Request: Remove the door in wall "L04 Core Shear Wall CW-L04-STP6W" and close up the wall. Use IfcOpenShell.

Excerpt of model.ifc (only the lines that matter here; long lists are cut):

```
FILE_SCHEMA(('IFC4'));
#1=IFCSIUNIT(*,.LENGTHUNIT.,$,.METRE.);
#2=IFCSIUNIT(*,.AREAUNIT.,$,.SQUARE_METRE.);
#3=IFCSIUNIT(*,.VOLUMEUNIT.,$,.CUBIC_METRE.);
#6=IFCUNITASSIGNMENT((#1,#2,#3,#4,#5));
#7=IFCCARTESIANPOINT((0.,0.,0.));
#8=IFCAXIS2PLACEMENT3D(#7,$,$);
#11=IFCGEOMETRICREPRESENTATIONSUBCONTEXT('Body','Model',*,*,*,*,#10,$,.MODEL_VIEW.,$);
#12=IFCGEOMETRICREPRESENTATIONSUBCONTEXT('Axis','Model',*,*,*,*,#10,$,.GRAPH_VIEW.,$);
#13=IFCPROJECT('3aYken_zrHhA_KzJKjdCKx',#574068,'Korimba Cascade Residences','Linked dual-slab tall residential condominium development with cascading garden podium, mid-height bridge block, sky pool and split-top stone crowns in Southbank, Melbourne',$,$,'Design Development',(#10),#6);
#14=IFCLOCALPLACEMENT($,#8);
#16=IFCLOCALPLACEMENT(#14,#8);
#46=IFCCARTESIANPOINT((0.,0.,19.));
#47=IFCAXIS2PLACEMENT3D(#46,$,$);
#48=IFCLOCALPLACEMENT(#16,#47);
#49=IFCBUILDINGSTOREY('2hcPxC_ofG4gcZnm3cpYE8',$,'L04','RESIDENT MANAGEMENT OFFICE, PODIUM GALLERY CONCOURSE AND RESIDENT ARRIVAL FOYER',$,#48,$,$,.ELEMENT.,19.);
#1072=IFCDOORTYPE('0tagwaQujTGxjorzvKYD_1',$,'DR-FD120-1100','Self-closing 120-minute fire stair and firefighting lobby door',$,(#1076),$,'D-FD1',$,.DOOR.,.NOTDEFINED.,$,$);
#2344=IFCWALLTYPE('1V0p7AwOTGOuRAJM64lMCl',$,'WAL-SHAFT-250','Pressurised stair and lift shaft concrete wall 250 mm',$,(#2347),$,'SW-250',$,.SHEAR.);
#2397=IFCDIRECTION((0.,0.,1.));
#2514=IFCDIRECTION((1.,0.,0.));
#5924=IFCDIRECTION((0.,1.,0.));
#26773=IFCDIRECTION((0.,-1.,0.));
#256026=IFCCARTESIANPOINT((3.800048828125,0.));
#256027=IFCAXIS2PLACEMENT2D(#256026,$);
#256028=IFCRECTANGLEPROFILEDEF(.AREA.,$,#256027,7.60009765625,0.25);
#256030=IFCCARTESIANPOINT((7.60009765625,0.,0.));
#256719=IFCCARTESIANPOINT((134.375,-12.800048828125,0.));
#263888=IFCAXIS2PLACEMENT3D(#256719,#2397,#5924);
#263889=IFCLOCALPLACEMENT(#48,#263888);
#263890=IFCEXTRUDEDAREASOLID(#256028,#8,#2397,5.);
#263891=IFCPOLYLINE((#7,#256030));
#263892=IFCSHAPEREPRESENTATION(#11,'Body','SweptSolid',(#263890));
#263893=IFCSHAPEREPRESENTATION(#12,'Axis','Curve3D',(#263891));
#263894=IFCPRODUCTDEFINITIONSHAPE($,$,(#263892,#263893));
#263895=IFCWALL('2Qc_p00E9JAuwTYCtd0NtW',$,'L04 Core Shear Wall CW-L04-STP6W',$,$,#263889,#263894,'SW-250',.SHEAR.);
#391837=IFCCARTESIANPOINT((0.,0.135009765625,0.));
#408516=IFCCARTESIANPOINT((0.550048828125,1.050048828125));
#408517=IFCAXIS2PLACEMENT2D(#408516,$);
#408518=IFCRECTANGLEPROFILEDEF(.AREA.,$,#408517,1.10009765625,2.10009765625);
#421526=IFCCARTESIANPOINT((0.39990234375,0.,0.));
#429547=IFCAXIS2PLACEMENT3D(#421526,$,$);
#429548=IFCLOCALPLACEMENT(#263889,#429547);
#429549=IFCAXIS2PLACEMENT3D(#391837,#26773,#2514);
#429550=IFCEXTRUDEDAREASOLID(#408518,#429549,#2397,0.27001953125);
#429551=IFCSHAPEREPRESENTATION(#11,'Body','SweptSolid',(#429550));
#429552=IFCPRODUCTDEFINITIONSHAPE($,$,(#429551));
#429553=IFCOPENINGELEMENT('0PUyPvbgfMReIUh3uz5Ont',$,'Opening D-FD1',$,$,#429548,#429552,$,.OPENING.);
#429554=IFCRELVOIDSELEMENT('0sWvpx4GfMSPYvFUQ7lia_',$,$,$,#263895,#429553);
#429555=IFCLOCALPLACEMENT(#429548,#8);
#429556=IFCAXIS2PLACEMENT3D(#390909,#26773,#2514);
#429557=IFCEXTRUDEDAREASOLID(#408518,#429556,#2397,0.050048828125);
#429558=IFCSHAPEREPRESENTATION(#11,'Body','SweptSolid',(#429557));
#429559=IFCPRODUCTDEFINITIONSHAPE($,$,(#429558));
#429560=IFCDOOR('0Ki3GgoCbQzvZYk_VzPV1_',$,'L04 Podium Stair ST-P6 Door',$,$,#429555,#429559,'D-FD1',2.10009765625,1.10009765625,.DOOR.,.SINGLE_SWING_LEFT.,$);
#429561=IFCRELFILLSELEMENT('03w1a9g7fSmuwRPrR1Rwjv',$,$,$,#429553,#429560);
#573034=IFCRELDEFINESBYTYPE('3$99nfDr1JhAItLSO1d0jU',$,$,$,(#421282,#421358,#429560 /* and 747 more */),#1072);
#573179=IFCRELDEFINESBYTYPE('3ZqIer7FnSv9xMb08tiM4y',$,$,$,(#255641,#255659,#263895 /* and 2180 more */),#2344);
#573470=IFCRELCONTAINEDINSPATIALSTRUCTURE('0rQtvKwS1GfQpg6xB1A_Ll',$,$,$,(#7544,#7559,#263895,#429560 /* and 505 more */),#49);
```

```python
import ifcopenshell
import ifcopenshell.api.feature
import ifcopenshell.api.root
import ifcopenshell.geom
import ifcopenshell.util.shape

model = ifcopenshell.open("model.ifc")
settings = ifcopenshell.geom.settings()


def volume(element):
    """Net volume in cubic metres, openings subtracted."""
    shape = ifcopenshell.geom.create_shape(settings, element)
    return ifcopenshell.util.shape.get_volume(shape.geometry)


door = model.by_guid("0Ki3GgoCbQzvZYk_VzPV1_")
opening = door.FillsVoids[0].RelatingOpeningElement
wall = opening.VoidsElements[0].RelatingBuildingElement
before = volume(wall)

ifcopenshell.api.root.remove_product(model, product=door)
ifcopenshell.api.feature.remove_feature(model, feature=opening)

after = volume(wall)

print(f"wall volume {before:.3f} -> {after:.3f} m3")

model.write("model_edited.ifc")
```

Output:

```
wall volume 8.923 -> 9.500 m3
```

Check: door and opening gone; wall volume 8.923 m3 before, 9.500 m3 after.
